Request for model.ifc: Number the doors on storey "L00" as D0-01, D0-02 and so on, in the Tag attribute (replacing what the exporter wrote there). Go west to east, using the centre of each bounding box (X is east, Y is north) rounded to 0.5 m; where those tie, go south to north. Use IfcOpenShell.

First a look at what the model holds.

```python
import ifcopenshell
import ifcopenshell.util.element
import ifcopenshell.util.placement

model = ifcopenshell.open("model.ifc")
print(model.schema)
storey = next(s for s in model.by_type("IfcBuildingStorey") if s.Name == "L00")
doors = [e for e in ifcopenshell.util.element.get_decomposition(storey) if e.is_a("IfcDoor")]
for e in sorted(doors, key=lambda e: e.id()):
    origin = ifcopenshell.util.placement.get_local_placement(e.ObjectPlacement)[:3, 3]
    print(e.id(), e.Tag, e.Name, origin.round(2) + 0.0, sep=" | ")
```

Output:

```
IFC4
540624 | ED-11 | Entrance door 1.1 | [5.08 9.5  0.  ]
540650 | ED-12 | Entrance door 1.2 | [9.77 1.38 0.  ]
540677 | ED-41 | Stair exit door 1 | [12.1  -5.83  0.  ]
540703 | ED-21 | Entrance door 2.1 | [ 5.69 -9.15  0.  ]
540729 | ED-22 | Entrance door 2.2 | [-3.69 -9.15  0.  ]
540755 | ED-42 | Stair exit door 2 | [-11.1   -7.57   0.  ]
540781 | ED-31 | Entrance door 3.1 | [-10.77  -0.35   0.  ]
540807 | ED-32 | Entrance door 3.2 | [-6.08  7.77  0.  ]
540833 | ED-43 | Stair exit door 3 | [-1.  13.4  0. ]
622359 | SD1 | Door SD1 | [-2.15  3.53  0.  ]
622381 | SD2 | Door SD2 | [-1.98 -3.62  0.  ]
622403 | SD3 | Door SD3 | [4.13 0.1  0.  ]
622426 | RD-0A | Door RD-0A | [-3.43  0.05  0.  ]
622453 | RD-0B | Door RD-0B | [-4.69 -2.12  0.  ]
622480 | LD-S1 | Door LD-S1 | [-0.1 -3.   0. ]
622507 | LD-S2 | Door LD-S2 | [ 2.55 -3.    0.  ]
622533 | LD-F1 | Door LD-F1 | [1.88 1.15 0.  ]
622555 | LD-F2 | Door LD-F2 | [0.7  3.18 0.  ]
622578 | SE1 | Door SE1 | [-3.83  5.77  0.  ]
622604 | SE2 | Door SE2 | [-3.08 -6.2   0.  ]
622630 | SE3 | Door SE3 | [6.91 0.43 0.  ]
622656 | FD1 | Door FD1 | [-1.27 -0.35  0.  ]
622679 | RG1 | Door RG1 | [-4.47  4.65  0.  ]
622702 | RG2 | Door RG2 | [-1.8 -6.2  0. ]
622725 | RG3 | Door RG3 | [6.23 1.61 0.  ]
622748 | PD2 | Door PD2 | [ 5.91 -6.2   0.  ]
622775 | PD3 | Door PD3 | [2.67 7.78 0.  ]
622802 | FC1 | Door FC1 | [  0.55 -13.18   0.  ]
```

```python
import ifcopenshell
import ifcopenshell.geom
import ifcopenshell.util.element
import ifcopenshell.util.shape

model = ifcopenshell.open("model.ifc")
settings = ifcopenshell.geom.settings()
settings.set("use-world-coords", True)


def centre(element):
    shape = ifcopenshell.geom.create_shape(settings, element)
    return ifcopenshell.util.shape.get_bbox_centroid(shape.geometry)


storey = next(s for s in model.by_type("IfcBuildingStorey") if s.Name == "L00")
doors = [e for e in ifcopenshell.util.element.get_decomposition(storey) if e.is_a("IfcDoor")]

# Insertion points can sit at a corner or the storey origin, so sort by the geometry (in metres).
centres = {e: centre(e) for e in doors}
doors.sort(key=lambda e: (round(centres[e][0] / 0.5), centres[e][1]))

for i, e in enumerate(doors, start=1):
    number = f"D0-{i:02d}"
    e.Tag = number
    print(e.id(), number)

model.write("model_edited.ifc")
```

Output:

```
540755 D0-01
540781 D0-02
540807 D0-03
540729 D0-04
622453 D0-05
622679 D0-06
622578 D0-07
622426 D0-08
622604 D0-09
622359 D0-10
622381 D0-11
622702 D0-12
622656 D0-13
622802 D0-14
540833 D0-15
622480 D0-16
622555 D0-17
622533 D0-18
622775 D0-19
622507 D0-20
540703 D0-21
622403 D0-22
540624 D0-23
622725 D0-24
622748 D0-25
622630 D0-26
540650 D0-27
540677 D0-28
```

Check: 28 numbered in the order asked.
